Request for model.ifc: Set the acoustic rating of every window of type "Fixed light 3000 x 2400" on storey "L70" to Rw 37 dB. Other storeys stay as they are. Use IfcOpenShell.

First a look at what the model holds.

```python
import ifcopenshell
import ifcopenshell.util.element

model = ifcopenshell.open("model.ifc")
print(model.schema)
storey = next(s for s in model.by_type("IfcBuildingStorey") if s.Name == "L70")
windows = [e for e in ifcopenshell.util.element.get_decomposition(storey) if e.is_a("IfcWindow")]
seen = {}
for e in windows:
    element_type = ifcopenshell.util.element.get_type(e)
    key = (element_type.Name if element_type != e and element_type else None, ifcopenshell.util.element.get_pset(e, "Pset_WindowCommon", "AcousticRating"))
    seen[key] = seen.get(key, 0) + 1
for (name, value), count in sorted(seen.items(), key=str):
    print(count, "x", name, "|", value)
```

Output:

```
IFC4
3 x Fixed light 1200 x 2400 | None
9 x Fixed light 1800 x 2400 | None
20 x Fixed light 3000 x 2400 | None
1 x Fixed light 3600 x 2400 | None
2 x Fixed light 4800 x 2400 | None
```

```python
import ifcopenshell
import ifcopenshell.api.pset
import ifcopenshell.util.element

model = ifcopenshell.open("model.ifc")

storey = next(s for s in model.by_type("IfcBuildingStorey") if s.Name == "L70")
windows = [e for e in ifcopenshell.util.element.get_decomposition(storey) if e.is_a("IfcWindow")]

count = 0
for e in windows:
    element_type = ifcopenshell.util.element.get_type(e)
    if element_type in (None, e) or element_type.Name != "Fixed light 3000 x 2400":
        continue
    found = ifcopenshell.util.element.get_pset(e, "Pset_WindowCommon", should_inherit=False)
    if found:
        pset = model.by_id(found["id"])
        if len(ifcopenshell.util.element.get_elements_by_pset(pset)) > 1:
            pset = ifcopenshell.api.pset.unshare_pset(model, products=[e], pset=pset)[0]
    else:
        pset = ifcopenshell.api.pset.add_pset(model, product=e, name="Pset_WindowCommon")
    ifcopenshell.api.pset.edit_pset(model, pset=pset, properties={"AcousticRating": "Rw 37 dB"})
    count += 1

print(count, "windows updated")

model.write("model_v2.ifc")
```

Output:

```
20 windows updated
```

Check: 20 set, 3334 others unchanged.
